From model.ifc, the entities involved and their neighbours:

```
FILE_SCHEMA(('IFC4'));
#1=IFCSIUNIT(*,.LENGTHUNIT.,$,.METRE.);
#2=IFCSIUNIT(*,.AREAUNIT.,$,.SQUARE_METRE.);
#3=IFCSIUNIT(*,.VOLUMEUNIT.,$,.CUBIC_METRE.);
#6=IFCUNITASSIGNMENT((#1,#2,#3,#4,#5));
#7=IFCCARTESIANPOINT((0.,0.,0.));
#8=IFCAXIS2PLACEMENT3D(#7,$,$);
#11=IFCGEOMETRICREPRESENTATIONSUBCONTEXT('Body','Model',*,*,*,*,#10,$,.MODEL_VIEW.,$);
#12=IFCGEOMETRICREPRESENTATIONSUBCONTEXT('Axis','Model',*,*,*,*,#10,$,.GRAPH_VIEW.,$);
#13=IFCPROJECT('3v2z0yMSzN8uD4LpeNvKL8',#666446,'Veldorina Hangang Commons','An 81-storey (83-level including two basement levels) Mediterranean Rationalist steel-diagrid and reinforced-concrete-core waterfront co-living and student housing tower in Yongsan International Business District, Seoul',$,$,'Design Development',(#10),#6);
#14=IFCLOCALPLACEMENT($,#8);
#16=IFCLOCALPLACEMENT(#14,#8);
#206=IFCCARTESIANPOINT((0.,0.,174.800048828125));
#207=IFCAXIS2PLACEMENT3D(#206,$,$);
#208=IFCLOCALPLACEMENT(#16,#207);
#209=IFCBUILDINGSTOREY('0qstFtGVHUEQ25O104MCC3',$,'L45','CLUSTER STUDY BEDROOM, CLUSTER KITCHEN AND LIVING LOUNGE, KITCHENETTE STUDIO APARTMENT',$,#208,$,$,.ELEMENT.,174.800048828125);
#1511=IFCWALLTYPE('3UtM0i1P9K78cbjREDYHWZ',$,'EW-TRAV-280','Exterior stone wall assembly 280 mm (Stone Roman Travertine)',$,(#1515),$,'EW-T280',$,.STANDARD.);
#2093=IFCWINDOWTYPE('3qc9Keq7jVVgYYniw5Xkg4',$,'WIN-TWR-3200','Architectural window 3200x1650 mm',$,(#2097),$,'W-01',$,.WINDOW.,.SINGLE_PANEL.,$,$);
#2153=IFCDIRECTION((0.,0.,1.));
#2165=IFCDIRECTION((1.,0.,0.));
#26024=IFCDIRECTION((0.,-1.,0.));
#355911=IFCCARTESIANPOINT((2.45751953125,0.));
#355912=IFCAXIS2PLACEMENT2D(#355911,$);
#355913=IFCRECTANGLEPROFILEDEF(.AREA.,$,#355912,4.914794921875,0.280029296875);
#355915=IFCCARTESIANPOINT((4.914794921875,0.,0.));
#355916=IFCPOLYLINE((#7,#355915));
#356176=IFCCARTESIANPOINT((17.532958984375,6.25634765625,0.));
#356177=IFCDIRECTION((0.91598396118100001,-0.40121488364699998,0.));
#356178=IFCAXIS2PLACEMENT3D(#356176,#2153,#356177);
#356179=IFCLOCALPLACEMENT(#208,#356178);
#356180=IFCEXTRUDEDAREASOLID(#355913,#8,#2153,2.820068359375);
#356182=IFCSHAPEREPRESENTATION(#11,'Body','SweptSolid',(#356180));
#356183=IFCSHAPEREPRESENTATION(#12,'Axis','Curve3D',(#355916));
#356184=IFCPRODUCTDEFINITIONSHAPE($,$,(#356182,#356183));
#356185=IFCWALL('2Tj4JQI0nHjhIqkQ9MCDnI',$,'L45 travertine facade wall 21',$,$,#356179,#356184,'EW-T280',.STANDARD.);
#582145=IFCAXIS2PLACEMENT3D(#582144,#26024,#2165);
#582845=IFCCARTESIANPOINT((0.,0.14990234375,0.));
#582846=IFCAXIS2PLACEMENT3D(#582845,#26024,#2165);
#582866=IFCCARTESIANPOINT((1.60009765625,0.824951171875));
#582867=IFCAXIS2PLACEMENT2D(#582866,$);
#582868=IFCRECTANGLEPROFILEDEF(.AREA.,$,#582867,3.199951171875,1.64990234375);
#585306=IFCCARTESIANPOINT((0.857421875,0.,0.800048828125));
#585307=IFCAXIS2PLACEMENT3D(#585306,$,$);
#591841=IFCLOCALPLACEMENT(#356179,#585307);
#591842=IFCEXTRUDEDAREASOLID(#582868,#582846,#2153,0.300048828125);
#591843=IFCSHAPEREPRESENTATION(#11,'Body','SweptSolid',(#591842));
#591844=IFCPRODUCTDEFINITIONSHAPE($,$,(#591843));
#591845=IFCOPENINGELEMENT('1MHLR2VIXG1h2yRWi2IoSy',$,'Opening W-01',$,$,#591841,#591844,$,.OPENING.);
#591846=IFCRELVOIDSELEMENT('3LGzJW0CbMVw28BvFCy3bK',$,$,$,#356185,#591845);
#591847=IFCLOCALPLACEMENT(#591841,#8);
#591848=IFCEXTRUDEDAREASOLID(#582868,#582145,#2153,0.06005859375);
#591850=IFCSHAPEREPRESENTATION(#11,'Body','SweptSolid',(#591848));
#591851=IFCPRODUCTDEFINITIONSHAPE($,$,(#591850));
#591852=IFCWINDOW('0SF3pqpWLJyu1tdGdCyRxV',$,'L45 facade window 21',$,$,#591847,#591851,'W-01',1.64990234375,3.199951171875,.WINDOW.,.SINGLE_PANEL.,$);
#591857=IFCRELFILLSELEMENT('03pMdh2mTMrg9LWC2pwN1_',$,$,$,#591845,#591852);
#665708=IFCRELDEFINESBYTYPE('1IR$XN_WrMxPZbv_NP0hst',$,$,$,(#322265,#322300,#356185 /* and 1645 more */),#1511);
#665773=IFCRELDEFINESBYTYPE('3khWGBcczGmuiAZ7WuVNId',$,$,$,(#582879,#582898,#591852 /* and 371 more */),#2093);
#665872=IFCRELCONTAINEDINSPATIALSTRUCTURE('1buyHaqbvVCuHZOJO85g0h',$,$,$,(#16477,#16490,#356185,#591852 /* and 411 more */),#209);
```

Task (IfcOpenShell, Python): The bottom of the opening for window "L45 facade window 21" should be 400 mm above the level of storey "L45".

```python
import numpy as np
import ifcopenshell
import ifcopenshell.api.geometry
import ifcopenshell.geom
import ifcopenshell.util.element
import ifcopenshell.util.placement
import ifcopenshell.util.shape
import ifcopenshell.util.unit

model = ifcopenshell.open("model.ifc")
unit_scale = ifcopenshell.util.unit.calculate_unit_scale(model)

window = model.by_guid("0SF3pqpWLJyu1tdGdCyRxV")
opening = window.FillsVoids[0].RelatingOpeningElement
storey = ifcopenshell.util.element.get_container(window, ifc_class="IfcBuildingStorey")
level = ifcopenshell.util.placement.get_local_placement(storey.ObjectPlacement)[2, 3]

# The opening's origin need not be at the sill, so measure its lowest point.
shape = ifcopenshell.geom.create_shape(ifcopenshell.geom.settings(), opening)
bottom = ifcopenshell.util.shape.get_shape_bottom_elevation(shape, shape.geometry) / unit_scale
dz = level + 0.4 - bottom

shift = np.array([0.0, 0.0, dz])
# The window is placed relative to its opening, so it follows when the opening moves.
matrix = ifcopenshell.util.placement.get_local_placement(opening.ObjectPlacement)
matrix[:3, 3] += shift
ifcopenshell.api.geometry.edit_object_placement(
    model, product=opening, matrix=matrix, is_si=False, should_transform_children=True
)

print(f"moved by {dz * unit_scale:+.3f} m")

model.write("model_edited.ifc")
```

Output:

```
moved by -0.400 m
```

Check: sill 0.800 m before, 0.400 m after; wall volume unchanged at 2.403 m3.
